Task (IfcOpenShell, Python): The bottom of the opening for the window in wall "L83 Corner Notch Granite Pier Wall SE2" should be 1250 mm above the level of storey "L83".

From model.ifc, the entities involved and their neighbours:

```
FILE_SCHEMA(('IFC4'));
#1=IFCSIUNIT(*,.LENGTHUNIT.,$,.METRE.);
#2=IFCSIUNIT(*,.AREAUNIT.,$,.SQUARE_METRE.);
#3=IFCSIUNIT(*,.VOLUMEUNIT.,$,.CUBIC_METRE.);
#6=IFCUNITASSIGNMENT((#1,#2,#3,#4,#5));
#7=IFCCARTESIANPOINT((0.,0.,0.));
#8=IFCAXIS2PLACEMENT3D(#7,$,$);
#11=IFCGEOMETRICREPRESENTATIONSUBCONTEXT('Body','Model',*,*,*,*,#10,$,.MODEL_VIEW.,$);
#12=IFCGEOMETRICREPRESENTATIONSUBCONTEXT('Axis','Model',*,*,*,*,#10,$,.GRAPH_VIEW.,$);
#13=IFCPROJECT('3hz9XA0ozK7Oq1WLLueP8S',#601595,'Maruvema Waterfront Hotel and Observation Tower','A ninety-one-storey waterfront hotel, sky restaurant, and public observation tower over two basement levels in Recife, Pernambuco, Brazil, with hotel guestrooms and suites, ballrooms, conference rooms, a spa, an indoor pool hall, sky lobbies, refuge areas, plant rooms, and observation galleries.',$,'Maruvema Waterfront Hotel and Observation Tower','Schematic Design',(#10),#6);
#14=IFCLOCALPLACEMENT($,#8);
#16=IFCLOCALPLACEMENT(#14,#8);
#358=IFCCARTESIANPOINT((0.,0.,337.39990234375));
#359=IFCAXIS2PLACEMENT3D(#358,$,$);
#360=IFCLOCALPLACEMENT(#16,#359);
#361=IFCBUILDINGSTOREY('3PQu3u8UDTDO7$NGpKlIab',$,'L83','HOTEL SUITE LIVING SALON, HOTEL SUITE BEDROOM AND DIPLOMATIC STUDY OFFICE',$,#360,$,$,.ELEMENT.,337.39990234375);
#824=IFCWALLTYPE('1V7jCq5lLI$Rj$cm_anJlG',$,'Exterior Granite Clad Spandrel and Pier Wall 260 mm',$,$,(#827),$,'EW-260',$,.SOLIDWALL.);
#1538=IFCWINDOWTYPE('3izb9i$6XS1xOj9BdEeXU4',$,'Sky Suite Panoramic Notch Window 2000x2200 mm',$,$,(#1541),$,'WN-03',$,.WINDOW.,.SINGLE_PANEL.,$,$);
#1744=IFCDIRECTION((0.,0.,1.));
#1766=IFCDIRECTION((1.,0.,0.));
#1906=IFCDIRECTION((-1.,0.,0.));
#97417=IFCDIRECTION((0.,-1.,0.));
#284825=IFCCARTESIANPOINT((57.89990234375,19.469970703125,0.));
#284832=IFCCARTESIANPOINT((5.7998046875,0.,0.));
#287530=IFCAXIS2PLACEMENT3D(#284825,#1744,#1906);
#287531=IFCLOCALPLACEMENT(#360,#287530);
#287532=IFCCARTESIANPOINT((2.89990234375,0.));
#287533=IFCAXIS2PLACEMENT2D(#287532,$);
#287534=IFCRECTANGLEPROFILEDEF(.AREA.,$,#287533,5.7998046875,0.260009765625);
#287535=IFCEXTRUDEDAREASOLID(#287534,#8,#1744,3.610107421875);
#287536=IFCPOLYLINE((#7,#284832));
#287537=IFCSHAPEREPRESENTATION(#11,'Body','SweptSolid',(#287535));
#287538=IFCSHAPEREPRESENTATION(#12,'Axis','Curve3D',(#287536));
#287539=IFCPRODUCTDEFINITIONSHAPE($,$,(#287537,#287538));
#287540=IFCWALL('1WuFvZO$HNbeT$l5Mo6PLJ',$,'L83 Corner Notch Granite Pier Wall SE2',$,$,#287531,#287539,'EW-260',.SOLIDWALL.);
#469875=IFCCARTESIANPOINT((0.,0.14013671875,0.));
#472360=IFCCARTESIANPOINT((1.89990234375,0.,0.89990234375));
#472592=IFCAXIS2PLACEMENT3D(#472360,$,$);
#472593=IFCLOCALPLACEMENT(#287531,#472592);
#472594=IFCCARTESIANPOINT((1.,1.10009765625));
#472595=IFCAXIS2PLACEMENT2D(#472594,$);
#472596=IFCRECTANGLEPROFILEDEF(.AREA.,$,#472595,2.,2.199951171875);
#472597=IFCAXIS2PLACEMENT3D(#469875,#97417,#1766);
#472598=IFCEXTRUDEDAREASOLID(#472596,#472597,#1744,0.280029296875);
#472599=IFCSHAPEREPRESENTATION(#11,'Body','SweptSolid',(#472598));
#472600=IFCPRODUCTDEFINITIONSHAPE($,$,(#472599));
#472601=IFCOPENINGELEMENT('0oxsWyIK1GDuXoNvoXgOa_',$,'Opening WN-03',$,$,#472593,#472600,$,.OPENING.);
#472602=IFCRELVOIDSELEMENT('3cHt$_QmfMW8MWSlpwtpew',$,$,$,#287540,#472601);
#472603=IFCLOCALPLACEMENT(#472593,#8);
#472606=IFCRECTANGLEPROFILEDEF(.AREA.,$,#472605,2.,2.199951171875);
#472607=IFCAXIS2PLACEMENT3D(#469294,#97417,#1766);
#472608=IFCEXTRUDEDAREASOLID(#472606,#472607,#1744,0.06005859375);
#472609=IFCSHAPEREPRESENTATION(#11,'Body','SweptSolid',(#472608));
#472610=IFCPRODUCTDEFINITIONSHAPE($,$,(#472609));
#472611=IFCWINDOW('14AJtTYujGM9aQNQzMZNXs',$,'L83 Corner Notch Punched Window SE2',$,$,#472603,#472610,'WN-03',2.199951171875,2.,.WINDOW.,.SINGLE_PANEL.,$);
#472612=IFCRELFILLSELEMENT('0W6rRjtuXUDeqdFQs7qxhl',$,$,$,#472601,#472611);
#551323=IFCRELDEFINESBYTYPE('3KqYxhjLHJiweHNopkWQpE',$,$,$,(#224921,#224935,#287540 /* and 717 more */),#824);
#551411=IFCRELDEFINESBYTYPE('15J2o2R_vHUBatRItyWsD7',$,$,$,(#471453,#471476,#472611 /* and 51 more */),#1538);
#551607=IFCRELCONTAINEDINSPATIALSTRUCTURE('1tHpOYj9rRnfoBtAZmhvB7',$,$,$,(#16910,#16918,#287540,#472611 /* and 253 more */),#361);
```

```python
import numpy as np
import ifcopenshell
import ifcopenshell.api.geometry
import ifcopenshell.geom
import ifcopenshell.util.element
import ifcopenshell.util.placement
import ifcopenshell.util.shape
import ifcopenshell.util.unit

model = ifcopenshell.open("model.ifc")
unit_scale = ifcopenshell.util.unit.calculate_unit_scale(model)

window = model.by_id(472611)
opening = window.FillsVoids[0].RelatingOpeningElement
storey = ifcopenshell.util.element.get_container(window, ifc_class="IfcBuildingStorey")
level = ifcopenshell.util.placement.get_local_placement(storey.ObjectPlacement)[2, 3]

# The opening's origin need not be at the sill, so measure its lowest point.
shape = ifcopenshell.geom.create_shape(ifcopenshell.geom.settings(), opening)
bottom = ifcopenshell.util.shape.get_shape_bottom_elevation(shape, shape.geometry) / unit_scale
dz = level + 1.25 / unit_scale - bottom

shift = np.array([0.0, 0.0, dz])
# The window is placed relative to its opening, so it follows when the opening moves.
matrix = ifcopenshell.util.placement.get_local_placement(opening.ObjectPlacement)
matrix[:3, 3] += shift
ifcopenshell.api.geometry.edit_object_placement(
    model, product=opening, matrix=matrix, is_si=False, should_transform_children=True
)

print(f"moved by {dz * unit_scale:+.3f} m")

model.write("model_updated.ifc")
```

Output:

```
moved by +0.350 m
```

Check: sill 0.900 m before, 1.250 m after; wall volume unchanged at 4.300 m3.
